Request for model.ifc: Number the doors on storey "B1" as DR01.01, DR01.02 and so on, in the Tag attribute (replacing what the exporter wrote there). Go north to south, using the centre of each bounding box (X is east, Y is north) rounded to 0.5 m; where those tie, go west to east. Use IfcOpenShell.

First a look at what the model holds.

```python
import ifcopenshell
import ifcopenshell.util.element
import ifcopenshell.util.placement

model = ifcopenshell.open("model.ifc")
print(model.schema)
storey = next(s for s in model.by_type("IfcBuildingStorey") if s.Name == "B1")
doors = [e for e in ifcopenshell.util.element.get_decomposition(storey) if e.is_a("IfcDoor")]
for e in sorted(doors, key=lambda e: e.id()):
    origin = ifcopenshell.util.placement.get_local_placement(e.ObjectPlacement)[:3, 3]
    print(e.id(), e.Tag, e.Name, origin.round(2) + 0.0, sep=" | ")
```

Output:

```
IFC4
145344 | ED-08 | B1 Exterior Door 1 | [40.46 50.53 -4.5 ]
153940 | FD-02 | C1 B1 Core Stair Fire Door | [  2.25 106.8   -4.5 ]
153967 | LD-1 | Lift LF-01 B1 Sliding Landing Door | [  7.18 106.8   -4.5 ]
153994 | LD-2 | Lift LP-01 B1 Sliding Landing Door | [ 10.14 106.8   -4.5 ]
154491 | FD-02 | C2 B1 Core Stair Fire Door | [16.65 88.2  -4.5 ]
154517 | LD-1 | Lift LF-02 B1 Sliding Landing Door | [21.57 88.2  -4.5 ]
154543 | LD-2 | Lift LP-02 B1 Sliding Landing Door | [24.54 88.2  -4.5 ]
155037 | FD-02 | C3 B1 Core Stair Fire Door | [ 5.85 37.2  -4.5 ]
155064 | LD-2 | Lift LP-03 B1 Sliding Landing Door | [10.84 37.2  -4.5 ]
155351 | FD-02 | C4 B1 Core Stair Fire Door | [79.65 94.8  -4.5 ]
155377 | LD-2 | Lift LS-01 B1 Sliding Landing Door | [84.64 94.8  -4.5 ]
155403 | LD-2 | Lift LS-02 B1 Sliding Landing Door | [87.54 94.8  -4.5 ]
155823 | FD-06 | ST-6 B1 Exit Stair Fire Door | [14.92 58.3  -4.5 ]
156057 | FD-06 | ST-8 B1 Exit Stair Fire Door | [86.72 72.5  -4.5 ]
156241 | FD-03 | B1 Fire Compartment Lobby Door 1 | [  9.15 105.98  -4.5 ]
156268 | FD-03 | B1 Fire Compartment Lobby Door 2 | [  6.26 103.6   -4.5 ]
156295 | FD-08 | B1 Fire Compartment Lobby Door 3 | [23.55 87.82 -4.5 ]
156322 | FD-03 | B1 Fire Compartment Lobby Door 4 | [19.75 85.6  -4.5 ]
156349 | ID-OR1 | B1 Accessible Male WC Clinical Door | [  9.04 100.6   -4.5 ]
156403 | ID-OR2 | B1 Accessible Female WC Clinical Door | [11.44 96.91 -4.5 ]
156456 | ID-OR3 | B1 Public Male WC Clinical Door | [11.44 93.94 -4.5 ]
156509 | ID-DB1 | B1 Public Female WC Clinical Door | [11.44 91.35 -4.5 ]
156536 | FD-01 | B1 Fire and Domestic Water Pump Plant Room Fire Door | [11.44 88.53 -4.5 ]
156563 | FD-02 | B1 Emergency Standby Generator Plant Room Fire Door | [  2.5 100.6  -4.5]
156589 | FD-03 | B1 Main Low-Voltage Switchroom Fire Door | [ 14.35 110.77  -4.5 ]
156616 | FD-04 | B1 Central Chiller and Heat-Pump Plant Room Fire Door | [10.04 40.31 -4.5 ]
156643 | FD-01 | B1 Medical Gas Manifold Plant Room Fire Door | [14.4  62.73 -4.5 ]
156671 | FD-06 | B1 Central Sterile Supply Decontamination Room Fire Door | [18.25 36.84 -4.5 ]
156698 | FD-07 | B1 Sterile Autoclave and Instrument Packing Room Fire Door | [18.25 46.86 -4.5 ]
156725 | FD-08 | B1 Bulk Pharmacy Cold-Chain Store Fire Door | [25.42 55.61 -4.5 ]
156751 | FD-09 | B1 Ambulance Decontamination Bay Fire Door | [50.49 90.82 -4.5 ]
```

```python
import ifcopenshell
import ifcopenshell.geom
import ifcopenshell.util.element
import ifcopenshell.util.shape

model = ifcopenshell.open("model.ifc")
settings = ifcopenshell.geom.settings()
settings.set("use-world-coords", True)


def centre(element):
    shape = ifcopenshell.geom.create_shape(settings, element)
    return ifcopenshell.util.shape.get_bbox_centroid(shape.geometry)


storey = next(s for s in model.by_type("IfcBuildingStorey") if s.Name == "B1")
doors = [e for e in ifcopenshell.util.element.get_decomposition(storey) if e.is_a("IfcDoor")]

# Insertion points can sit at a corner or the storey origin, so sort by the geometry (in metres).
centres = {e: centre(e) for e in doors}
doors.sort(key=lambda e: (-round(centres[e][1] / 0.5), centres[e][0]))

for i, e in enumerate(doors, start=1):
    number = f"DR01.{i:02d}"
    e.Tag = number
    print(e.id(), number)

model.write("model_updated.ifc")
```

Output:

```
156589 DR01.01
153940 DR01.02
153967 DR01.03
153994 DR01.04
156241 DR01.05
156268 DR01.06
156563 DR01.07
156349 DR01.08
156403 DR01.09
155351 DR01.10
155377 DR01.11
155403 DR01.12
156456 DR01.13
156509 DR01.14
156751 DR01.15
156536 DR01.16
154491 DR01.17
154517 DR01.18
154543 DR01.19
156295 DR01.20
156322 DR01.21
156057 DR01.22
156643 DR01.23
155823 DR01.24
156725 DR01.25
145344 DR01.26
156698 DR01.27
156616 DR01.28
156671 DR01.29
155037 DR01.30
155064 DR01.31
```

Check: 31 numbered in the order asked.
